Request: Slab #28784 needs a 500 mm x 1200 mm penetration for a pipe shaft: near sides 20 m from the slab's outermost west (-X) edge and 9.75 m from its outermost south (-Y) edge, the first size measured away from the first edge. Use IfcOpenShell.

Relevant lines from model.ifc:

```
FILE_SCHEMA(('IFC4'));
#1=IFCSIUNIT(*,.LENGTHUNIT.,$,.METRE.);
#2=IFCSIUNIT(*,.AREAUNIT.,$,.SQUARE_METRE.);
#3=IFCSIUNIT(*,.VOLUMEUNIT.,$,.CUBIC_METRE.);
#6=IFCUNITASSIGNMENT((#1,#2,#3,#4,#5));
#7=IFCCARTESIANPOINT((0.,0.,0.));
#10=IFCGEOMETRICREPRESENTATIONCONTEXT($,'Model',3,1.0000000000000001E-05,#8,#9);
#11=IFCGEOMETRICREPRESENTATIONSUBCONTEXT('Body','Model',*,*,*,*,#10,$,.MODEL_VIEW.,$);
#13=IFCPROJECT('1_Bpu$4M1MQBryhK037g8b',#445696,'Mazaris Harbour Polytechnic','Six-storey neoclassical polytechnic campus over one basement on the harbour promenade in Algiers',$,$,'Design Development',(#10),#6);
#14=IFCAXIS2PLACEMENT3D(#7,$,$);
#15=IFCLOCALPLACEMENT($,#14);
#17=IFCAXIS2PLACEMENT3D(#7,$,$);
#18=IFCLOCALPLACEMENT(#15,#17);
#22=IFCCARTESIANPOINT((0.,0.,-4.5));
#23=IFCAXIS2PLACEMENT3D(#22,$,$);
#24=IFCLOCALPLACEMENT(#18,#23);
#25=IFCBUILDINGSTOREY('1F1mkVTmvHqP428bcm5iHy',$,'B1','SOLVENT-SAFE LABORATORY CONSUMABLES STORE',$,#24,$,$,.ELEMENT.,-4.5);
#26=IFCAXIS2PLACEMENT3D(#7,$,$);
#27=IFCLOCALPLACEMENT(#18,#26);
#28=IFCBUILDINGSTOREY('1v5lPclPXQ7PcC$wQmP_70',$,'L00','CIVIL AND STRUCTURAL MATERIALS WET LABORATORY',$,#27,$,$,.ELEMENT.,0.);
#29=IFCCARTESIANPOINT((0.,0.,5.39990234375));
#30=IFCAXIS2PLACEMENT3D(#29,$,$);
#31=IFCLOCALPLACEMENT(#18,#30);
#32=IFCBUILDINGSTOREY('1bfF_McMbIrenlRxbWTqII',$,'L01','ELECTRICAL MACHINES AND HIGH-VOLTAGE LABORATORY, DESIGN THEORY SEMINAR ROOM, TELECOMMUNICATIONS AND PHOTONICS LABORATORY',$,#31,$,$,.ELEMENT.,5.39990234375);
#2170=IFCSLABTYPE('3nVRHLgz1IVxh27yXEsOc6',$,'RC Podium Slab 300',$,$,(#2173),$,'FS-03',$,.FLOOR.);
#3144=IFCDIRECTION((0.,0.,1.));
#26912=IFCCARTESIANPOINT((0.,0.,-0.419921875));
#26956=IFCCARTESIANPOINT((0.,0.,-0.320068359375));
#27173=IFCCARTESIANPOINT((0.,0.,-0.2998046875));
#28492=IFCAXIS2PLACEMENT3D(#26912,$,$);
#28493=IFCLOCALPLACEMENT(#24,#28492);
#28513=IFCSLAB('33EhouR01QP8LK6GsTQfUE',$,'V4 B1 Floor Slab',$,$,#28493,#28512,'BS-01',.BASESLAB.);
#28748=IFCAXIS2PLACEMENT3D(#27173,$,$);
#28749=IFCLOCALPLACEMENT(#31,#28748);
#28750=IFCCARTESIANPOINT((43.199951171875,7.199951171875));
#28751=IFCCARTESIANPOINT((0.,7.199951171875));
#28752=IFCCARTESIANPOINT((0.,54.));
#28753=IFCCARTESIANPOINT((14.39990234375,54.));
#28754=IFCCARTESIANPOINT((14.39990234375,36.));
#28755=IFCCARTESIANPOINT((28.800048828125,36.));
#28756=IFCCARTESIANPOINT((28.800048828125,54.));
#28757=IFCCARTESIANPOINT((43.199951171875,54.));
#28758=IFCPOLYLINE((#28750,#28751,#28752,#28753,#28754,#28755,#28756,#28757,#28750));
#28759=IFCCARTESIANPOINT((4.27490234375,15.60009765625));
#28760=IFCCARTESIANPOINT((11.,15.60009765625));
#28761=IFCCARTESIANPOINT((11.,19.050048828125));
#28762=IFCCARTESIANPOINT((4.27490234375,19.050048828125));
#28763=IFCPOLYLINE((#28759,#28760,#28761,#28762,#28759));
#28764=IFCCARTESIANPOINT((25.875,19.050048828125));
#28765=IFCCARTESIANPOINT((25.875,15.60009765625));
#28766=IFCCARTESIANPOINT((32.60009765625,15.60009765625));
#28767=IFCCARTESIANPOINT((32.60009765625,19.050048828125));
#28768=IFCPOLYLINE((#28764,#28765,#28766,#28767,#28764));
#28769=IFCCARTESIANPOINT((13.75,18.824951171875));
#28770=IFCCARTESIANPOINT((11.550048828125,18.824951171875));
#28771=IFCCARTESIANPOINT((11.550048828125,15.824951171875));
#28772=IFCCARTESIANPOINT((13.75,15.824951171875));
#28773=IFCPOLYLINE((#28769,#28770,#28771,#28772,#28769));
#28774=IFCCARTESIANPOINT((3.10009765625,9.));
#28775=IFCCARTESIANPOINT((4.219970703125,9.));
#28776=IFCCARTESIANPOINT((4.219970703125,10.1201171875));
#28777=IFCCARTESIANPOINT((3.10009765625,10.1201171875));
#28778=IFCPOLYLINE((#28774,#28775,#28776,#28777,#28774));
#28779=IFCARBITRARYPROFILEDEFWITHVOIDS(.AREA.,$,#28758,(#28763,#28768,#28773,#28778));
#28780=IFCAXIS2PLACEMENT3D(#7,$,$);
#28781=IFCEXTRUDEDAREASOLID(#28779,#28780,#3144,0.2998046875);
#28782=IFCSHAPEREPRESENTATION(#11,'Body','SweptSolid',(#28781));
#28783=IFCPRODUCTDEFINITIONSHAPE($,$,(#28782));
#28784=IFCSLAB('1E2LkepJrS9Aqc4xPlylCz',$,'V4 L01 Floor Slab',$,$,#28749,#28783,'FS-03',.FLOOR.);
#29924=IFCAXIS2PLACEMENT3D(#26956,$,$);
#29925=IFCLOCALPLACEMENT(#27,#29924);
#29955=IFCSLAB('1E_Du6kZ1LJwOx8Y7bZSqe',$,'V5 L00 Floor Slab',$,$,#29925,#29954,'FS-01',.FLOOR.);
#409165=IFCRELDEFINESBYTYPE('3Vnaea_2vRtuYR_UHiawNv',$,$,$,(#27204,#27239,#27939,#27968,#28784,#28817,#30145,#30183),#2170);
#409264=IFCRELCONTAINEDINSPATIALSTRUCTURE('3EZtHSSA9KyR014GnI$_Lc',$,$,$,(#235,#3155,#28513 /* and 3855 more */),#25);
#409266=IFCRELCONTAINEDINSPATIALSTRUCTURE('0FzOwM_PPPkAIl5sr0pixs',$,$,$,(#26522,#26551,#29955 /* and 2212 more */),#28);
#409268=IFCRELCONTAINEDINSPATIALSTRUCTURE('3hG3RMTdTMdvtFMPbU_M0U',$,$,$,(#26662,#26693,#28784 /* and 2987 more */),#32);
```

```python
import numpy as np
import ifcopenshell
import ifcopenshell.api.feature
import ifcopenshell.api.geometry
import ifcopenshell.api.root
import ifcopenshell.geom
import ifcopenshell.util.placement
import ifcopenshell.util.representation
import ifcopenshell.util.shape
import ifcopenshell.util.unit

model = ifcopenshell.open("model.ifc")
unit_scale = ifcopenshell.util.unit.calculate_unit_scale(model)
settings = ifcopenshell.geom.settings()


def volume(element):
    """Net volume in cubic metres, openings subtracted."""
    shape = ifcopenshell.geom.create_shape(settings, element)
    return ifcopenshell.util.shape.get_volume(shape.geometry)


slab = model.by_guid("1E2LkepJrS9Aqc4xPlylCz")
before = volume(slab)

# Extent in the slab's own axes, in metres. The edges named are its -X and -Y sides.
slab_shape = ifcopenshell.geom.create_shape(settings, slab)
vertices = ifcopenshell.util.shape.get_vertices(slab_shape.geometry)
x_min, y_min, bottom = vertices.min(axis=0)
top = vertices[:, 2].max()

opening = ifcopenshell.api.root.create_entity(model, ifc_class="IfcOpeningElement", name="Pipe shaft opening", predefined_type="OPENING")
context = ifcopenshell.util.representation.get_context(model, "Model", "Body", "MODEL_VIEW")
width, depth = 0.5, 1.2
outline = [(0.0, 0.0), (width, 0.0), (width, depth), (0.0, depth), (0.0, 0.0)]
# Overshoot both faces by 50 mm so the cut is clean.
shape = ifcopenshell.api.geometry.add_slab_representation(
    model, context=context, depth=top - bottom + 0.1, polyline=outline
)
ifcopenshell.api.geometry.assign_representation(model, product=opening, representation=shape)

matrix = ifcopenshell.util.placement.get_local_placement(slab.ObjectPlacement)
matrix[:, 3] = matrix @ np.append(np.array([x_min + 20, y_min + 9.75, bottom - 0.05]) / unit_scale, 1.0)
ifcopenshell.api.geometry.edit_object_placement(model, product=opening, matrix=matrix, is_si=False)
ifcopenshell.api.feature.add_feature(model, feature=opening, element=slab)

after = volume(slab)

print(f"slab volume {before:.3f} -> {after:.3f} m3")

model.write("model_v2.ifc")
```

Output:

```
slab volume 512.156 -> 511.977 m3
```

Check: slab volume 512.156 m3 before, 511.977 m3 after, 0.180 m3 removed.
